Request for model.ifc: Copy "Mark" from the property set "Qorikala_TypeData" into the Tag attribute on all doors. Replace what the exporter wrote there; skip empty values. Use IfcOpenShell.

First a look at what the model holds.

```python
import ifcopenshell
import ifcopenshell.util.element

model = ifcopenshell.open("model.ifc")
print(model.schema)
doors = model.by_type("IfcDoor")
print(len(doors), "doors")
for e in doors[:8]:
    source = ifcopenshell.util.element.get_pset(e, "Qorikala_TypeData", "Mark")
    target = e.Tag
    print(e.id(), repr(source), repr(target), sep=" | ")
```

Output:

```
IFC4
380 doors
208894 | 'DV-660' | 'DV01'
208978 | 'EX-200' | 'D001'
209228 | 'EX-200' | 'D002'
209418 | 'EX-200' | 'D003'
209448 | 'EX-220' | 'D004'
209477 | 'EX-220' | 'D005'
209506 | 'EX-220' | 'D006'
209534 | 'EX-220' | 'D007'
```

```python
import ifcopenshell
import ifcopenshell.util.element

model = ifcopenshell.open("model.ifc")

count = 0
for e in model.by_type("IfcDoor"):
    value = ifcopenshell.util.element.get_pset(e, "Qorikala_TypeData", "Mark")
    current = e.Tag
    if not value or not value.strip() or current == value:
        continue
    e.Tag = value
    count += 1

print(count, "doors updated")

model.write("model_rev.ifc")
```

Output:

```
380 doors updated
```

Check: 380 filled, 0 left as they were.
